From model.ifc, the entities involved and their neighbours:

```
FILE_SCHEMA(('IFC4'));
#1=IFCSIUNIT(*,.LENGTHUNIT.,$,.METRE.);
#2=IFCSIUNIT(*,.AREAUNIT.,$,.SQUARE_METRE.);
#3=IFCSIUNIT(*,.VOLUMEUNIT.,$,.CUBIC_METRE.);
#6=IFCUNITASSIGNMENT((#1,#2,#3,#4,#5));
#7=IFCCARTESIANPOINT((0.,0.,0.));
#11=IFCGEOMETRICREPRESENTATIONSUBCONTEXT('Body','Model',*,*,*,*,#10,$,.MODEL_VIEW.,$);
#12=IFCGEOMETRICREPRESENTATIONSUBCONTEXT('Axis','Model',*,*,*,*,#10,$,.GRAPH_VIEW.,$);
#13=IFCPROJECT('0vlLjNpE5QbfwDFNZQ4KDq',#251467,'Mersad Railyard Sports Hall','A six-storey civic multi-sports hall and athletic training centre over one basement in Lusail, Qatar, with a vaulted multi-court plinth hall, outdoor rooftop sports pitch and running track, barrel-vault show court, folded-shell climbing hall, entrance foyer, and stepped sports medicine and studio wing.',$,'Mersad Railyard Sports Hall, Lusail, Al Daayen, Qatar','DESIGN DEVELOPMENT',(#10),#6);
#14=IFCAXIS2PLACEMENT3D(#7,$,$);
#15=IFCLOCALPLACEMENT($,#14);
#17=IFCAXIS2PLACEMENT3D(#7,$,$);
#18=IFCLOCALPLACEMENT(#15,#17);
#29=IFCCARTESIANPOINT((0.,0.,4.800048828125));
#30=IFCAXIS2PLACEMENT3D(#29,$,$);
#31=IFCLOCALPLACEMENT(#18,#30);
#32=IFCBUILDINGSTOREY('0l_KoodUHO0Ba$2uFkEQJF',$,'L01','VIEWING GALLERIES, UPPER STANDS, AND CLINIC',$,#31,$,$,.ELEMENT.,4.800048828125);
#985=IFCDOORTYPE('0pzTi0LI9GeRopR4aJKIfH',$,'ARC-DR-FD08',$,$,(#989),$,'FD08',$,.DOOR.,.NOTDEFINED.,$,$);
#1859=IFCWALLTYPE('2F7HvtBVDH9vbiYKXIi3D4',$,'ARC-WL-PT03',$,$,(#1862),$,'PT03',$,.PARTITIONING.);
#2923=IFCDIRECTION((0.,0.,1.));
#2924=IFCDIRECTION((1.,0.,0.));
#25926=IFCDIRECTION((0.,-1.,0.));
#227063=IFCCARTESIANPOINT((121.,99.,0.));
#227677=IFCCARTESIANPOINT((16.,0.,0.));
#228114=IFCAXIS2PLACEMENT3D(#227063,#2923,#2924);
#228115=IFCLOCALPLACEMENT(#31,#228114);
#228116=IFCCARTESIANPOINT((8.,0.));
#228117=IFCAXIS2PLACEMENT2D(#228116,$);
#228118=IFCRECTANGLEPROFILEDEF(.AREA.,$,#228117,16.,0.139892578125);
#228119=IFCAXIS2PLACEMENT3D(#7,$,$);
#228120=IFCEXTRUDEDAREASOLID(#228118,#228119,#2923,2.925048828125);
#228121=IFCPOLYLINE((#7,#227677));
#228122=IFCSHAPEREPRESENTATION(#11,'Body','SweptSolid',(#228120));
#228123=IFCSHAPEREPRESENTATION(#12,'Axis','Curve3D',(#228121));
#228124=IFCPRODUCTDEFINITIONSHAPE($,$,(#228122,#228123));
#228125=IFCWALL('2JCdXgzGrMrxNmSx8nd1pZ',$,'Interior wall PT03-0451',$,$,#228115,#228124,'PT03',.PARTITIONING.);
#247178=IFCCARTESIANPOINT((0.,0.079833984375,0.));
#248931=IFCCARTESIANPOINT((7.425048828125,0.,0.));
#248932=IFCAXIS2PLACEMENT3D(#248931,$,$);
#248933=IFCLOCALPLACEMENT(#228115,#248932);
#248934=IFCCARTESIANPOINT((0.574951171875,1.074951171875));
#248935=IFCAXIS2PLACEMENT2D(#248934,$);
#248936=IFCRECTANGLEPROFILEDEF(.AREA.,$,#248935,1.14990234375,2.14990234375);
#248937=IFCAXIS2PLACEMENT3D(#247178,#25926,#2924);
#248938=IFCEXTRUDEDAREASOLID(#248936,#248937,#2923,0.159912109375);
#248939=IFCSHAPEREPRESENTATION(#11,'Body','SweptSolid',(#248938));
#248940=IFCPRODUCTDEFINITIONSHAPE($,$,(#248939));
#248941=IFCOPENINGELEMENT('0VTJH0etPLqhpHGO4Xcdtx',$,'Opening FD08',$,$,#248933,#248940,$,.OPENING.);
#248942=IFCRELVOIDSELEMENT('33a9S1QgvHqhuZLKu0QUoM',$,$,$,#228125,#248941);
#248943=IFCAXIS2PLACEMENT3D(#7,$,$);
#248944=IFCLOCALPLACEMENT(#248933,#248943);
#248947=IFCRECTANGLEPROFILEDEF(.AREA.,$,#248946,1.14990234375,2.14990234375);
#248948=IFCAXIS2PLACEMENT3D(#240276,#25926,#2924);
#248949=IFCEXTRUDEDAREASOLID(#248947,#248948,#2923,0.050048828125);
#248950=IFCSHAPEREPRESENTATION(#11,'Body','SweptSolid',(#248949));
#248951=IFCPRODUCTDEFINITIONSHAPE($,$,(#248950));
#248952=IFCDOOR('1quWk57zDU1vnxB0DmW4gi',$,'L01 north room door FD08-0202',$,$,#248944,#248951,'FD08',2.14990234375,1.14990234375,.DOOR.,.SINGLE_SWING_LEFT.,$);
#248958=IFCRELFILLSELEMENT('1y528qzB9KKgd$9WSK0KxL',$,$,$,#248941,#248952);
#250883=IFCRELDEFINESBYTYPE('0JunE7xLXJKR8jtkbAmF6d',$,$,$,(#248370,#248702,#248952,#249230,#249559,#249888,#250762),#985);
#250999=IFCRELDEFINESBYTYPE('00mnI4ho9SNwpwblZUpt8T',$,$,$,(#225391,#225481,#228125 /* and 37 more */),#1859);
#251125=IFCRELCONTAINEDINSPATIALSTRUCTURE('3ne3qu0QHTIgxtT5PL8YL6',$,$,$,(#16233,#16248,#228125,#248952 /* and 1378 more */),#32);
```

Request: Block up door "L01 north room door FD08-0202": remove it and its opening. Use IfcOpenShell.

```python
import ifcopenshell
import ifcopenshell.api.feature
import ifcopenshell.api.root
import ifcopenshell.geom
import ifcopenshell.util.shape

model = ifcopenshell.open("model.ifc")
settings = ifcopenshell.geom.settings()


def volume(element):
    """Net volume in cubic metres, openings subtracted."""
    shape = ifcopenshell.geom.create_shape(settings, element)
    return ifcopenshell.util.shape.get_volume(shape.geometry)


door = model.by_guid("1quWk57zDU1vnxB0DmW4gi")
opening = door.FillsVoids[0].RelatingOpeningElement
wall = opening.VoidsElements[0].RelatingBuildingElement
before = volume(wall)

ifcopenshell.api.root.remove_product(model, product=door)
ifcopenshell.api.feature.remove_feature(model, feature=opening)

after = volume(wall)

print(f"wall volume {before:.3f} -> {after:.3f} m3")

model.write("model_edited.ifc")
```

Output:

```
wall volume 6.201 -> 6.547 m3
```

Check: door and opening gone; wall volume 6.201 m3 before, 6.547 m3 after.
